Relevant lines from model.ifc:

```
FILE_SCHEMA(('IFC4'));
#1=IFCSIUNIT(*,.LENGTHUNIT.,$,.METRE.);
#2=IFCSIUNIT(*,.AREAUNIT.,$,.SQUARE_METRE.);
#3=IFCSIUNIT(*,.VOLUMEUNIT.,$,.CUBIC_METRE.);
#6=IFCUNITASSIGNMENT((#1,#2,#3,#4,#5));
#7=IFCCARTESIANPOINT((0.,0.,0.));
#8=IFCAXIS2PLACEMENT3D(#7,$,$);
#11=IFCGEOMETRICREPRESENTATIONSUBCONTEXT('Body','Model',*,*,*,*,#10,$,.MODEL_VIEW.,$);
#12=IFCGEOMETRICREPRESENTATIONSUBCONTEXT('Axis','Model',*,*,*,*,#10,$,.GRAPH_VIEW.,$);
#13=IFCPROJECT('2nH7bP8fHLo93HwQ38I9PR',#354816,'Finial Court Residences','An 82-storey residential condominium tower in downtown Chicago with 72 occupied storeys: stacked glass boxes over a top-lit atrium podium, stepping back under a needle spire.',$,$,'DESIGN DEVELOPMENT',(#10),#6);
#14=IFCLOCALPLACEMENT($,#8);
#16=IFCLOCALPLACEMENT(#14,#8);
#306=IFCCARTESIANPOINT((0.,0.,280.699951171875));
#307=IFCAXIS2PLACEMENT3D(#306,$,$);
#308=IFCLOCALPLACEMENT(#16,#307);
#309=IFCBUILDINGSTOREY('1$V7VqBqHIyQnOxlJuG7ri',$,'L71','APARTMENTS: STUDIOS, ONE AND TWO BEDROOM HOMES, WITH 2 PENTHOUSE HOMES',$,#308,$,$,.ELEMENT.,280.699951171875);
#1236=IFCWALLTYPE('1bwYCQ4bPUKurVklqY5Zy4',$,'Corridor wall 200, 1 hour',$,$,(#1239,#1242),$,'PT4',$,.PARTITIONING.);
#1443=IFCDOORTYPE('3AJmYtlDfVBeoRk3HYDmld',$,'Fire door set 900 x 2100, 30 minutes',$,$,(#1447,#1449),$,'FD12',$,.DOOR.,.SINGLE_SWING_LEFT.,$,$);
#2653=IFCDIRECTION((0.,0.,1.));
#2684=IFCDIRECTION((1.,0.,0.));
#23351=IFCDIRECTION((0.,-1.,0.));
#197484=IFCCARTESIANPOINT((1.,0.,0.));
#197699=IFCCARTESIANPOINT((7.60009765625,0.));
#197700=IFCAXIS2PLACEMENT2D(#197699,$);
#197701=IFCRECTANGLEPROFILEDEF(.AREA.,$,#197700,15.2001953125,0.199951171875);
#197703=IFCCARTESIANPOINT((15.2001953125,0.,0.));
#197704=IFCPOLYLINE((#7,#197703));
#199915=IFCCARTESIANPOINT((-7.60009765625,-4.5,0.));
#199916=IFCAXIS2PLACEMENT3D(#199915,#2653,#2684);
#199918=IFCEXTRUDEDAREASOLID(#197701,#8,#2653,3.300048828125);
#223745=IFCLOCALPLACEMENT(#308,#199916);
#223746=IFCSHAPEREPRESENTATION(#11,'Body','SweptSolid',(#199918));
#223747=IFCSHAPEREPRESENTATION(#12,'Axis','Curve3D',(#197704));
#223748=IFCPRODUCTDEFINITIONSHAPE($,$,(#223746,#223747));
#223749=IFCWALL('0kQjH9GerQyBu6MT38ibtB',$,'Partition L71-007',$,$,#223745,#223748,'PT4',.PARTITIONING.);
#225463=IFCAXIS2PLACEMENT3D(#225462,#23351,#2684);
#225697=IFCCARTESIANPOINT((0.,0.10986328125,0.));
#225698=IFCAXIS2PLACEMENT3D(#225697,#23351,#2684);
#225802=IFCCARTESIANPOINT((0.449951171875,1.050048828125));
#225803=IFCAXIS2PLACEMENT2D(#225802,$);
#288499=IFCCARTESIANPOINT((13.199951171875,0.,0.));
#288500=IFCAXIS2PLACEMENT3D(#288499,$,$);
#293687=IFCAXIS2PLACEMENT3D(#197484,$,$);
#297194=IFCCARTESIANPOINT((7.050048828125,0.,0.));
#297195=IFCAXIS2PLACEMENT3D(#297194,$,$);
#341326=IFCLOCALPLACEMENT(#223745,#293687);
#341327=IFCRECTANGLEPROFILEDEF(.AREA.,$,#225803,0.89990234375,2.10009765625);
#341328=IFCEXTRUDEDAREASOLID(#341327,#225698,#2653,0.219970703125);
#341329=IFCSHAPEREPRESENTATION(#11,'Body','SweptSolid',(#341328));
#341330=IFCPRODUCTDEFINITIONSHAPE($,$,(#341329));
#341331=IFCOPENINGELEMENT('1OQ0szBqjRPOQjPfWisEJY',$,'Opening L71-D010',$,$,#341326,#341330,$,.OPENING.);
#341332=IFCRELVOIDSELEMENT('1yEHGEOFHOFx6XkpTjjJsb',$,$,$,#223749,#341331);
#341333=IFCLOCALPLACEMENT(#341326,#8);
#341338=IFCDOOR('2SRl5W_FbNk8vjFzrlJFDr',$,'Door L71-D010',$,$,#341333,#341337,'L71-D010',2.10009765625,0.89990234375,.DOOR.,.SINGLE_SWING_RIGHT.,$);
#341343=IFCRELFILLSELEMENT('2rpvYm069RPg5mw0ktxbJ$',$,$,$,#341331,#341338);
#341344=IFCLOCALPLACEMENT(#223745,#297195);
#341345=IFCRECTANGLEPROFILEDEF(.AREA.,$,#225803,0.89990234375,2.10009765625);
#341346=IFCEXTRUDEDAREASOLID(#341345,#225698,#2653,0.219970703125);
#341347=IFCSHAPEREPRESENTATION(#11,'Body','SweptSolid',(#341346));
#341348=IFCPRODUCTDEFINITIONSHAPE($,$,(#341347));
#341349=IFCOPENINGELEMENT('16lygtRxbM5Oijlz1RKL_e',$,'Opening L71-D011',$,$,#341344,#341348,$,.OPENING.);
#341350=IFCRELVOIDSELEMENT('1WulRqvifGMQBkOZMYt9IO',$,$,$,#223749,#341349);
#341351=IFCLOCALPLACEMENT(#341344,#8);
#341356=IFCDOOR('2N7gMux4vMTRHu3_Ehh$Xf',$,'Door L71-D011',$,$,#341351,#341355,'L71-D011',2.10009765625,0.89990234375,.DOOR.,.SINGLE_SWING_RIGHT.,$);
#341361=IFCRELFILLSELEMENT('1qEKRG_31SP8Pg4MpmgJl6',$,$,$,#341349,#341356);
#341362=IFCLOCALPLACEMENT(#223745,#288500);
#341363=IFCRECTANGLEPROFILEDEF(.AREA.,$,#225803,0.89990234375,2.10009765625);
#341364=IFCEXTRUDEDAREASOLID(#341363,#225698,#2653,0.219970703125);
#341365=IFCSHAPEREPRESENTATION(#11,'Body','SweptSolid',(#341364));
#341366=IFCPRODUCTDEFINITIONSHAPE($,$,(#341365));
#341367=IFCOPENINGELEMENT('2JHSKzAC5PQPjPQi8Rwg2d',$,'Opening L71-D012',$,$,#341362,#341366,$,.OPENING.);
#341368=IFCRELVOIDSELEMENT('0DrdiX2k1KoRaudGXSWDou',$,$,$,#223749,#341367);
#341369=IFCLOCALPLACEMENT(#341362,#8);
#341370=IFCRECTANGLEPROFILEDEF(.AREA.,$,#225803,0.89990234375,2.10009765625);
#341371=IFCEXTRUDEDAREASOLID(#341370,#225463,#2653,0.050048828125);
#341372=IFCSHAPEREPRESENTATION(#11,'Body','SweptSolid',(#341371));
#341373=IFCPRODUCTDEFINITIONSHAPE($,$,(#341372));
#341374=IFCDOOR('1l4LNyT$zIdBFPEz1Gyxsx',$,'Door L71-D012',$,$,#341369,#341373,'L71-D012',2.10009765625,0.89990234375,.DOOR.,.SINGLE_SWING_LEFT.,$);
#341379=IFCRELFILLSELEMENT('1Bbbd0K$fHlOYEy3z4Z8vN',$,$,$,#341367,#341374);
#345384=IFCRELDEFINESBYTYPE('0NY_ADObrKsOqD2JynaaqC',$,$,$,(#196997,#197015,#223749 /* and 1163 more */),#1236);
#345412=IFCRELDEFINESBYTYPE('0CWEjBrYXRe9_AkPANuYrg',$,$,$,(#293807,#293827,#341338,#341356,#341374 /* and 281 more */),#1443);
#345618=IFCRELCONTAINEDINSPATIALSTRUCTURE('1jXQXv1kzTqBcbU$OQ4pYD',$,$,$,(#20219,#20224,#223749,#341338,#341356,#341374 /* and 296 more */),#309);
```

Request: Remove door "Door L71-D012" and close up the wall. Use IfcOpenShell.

```python
import ifcopenshell
import ifcopenshell.api.feature
import ifcopenshell.api.root
import ifcopenshell.geom
import ifcopenshell.util.shape

model = ifcopenshell.open("model.ifc")
settings = ifcopenshell.geom.settings()


def volume(element):
    """Net volume in cubic metres, openings subtracted."""
    shape = ifcopenshell.geom.create_shape(settings, element)
    return ifcopenshell.util.shape.get_volume(shape.geometry)


door = model.by_guid("1l4LNyT$zIdBFPEz1Gyxsx")
opening = door.FillsVoids[0].RelatingOpeningElement
wall = opening.VoidsElements[0].RelatingBuildingElement
before = volume(wall)

ifcopenshell.api.root.remove_product(model, product=door)
ifcopenshell.api.feature.remove_feature(model, feature=opening)

after = volume(wall)

print(f"wall volume {before:.3f} -> {after:.3f} m3")

model.write("model-out.ifc")
```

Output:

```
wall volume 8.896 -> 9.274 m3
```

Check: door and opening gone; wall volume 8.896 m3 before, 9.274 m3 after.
